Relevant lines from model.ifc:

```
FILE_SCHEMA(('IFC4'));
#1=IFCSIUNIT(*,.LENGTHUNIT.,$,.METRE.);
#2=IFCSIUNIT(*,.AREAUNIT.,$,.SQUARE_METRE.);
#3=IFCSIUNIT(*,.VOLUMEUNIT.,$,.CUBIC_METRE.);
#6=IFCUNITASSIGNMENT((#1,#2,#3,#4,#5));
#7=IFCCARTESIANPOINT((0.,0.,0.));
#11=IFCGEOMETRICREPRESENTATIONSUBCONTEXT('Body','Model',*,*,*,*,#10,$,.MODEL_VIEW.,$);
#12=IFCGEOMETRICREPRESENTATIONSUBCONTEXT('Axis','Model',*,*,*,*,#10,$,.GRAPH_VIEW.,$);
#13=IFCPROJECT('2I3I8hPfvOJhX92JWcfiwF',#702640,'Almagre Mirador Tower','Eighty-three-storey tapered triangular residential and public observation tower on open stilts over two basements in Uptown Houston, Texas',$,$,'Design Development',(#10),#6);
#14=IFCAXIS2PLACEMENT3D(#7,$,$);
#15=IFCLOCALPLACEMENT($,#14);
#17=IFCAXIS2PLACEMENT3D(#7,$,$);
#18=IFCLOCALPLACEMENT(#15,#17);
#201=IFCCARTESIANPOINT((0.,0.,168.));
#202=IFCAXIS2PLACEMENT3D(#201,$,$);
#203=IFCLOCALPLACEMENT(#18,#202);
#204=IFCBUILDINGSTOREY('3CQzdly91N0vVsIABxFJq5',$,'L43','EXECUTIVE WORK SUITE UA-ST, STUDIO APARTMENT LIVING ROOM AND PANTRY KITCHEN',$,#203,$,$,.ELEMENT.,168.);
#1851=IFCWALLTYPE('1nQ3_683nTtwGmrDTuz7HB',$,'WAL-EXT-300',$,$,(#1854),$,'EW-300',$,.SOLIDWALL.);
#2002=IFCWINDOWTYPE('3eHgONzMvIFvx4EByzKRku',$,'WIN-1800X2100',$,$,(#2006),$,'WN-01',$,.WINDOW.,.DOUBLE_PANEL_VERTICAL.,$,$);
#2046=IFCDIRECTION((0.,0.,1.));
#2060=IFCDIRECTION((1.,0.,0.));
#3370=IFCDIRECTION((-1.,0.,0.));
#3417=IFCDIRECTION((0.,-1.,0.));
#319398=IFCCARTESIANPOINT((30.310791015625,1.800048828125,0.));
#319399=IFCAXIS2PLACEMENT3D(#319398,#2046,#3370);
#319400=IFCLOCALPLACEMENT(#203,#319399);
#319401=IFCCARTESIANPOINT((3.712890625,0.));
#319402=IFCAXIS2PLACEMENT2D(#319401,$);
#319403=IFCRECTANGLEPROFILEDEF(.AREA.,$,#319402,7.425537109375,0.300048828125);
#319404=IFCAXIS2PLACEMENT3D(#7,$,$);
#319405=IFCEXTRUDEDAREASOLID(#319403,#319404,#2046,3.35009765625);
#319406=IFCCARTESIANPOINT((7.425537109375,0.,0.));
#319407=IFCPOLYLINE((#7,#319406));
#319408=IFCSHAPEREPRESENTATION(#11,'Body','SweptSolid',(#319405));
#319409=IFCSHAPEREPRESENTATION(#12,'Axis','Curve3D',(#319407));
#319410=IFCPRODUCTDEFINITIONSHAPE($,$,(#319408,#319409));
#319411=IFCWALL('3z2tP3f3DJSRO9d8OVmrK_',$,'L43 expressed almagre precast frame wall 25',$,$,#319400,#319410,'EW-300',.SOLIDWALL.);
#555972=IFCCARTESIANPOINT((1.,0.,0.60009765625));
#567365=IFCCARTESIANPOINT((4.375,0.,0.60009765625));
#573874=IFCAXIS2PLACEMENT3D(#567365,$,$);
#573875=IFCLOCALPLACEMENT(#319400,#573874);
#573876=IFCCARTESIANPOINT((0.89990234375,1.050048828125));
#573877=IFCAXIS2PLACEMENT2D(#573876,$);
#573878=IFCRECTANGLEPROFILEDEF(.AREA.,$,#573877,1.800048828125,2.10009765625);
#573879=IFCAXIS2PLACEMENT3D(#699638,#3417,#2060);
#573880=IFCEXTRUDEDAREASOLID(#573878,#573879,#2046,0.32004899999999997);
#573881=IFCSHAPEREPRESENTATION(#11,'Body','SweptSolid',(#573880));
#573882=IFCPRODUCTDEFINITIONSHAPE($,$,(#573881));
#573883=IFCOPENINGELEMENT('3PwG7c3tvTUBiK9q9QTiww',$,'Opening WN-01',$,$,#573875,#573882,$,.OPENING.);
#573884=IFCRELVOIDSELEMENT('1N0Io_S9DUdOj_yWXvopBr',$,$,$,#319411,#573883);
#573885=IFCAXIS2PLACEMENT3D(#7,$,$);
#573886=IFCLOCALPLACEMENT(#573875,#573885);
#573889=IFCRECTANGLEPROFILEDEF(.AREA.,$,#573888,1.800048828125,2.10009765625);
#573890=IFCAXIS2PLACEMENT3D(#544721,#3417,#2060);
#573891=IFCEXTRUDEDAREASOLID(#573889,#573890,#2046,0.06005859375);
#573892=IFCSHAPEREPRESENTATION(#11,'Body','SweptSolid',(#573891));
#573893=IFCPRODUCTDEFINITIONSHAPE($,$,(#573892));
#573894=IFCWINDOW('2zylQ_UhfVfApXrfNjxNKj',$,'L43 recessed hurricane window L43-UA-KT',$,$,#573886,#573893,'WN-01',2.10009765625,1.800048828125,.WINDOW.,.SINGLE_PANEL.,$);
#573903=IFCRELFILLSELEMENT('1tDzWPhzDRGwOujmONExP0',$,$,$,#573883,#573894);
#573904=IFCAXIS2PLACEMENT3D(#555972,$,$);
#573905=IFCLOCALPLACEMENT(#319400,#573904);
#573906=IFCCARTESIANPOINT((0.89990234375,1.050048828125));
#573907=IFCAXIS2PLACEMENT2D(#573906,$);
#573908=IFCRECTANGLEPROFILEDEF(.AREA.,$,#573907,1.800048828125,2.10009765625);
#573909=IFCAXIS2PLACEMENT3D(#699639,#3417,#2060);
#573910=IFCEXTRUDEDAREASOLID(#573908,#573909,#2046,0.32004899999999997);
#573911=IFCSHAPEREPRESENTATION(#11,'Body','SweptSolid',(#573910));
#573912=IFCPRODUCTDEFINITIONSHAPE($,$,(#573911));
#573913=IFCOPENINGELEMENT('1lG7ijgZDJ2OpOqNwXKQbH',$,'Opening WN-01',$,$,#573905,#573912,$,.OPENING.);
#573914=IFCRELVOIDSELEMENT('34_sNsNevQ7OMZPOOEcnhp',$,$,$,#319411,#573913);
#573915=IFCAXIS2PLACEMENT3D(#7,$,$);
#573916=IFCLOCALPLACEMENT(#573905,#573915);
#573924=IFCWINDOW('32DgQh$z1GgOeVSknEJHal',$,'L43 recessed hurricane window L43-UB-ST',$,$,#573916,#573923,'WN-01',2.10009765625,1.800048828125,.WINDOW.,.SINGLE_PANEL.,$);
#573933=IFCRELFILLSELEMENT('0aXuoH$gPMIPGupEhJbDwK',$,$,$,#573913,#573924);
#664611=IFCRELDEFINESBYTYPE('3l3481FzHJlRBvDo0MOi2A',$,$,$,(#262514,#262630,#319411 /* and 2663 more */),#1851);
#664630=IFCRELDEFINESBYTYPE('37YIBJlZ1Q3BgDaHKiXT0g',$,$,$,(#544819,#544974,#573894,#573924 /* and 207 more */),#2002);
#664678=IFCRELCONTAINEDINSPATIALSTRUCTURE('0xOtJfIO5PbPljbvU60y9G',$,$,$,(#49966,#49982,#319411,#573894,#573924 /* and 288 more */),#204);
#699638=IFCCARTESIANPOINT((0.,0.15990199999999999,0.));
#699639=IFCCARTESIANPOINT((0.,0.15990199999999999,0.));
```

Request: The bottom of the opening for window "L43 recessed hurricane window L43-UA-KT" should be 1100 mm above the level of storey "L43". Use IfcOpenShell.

```python
import numpy as np
import ifcopenshell
import ifcopenshell.api.geometry
import ifcopenshell.geom
import ifcopenshell.util.element
import ifcopenshell.util.placement
import ifcopenshell.util.shape
import ifcopenshell.util.unit

model = ifcopenshell.open("model.ifc")
unit_scale = ifcopenshell.util.unit.calculate_unit_scale(model)

window = model.by_guid("2zylQ_UhfVfApXrfNjxNKj")
opening = window.FillsVoids[0].RelatingOpeningElement
storey = ifcopenshell.util.element.get_container(window, ifc_class="IfcBuildingStorey")
level = ifcopenshell.util.placement.get_local_placement(storey.ObjectPlacement)[2, 3]

# The opening's origin need not be at the sill, so measure its lowest point.
shape = ifcopenshell.geom.create_shape(ifcopenshell.geom.settings(), opening)
bottom = ifcopenshell.util.shape.get_shape_bottom_elevation(shape, shape.geometry) / unit_scale
dz = level + 1.1 / unit_scale - bottom

shift = np.array([0.0, 0.0, dz])
# The window is placed relative to its opening, so it follows when the opening moves.
matrix = ifcopenshell.util.placement.get_local_placement(opening.ObjectPlacement)
matrix[:3, 3] += shift
ifcopenshell.api.geometry.edit_object_placement(
    model, product=opening, matrix=matrix, is_si=False, should_transform_children=True
)

print(f"moved by {dz * unit_scale:+.3f} m")

model.write("model_updated.ifc")
```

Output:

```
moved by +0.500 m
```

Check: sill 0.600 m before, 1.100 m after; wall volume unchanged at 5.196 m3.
